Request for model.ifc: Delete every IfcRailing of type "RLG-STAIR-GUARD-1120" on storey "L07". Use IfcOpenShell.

First a look at what the model holds.

```python
import ifcopenshell
import ifcopenshell.util.element

model = ifcopenshell.open("model.ifc")
print(model.schema)
storey = next(s for s in model.by_type("IfcBuildingStorey") if s.Name == "L07")
railings = [e for e in ifcopenshell.util.element.get_decomposition(storey) if e.is_a("IfcRailing")]
seen = {}
for e in railings:
    element_type = ifcopenshell.util.element.get_type(e)
    name = element_type.Name if element_type not in (None, e) else None
    seen[name] = seen.get(name, 0) + 1
for name, count in sorted(seen.items(), key=str):
    print(count, "x", name)
```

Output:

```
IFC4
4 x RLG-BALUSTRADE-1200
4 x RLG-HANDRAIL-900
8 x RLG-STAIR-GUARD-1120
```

```python
import ifcopenshell
import ifcopenshell.api.root
import ifcopenshell.util.element

model = ifcopenshell.open("model.ifc")

storey = next(s for s in model.by_type("IfcBuildingStorey") if s.Name == "L07")
railings = [e for e in ifcopenshell.util.element.get_decomposition(storey) if e.is_a("IfcRailing")]
targets = [e for e in railings if (t := ifcopenshell.util.element.get_type(e)) not in (None, e) and t.Name == "RLG-STAIR-GUARD-1120"]

for e in targets:
    ifcopenshell.api.root.remove_product(model, product=e)
print(len(targets), "removed")

model.write("model_v2.ifc")
```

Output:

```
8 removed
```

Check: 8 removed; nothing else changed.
